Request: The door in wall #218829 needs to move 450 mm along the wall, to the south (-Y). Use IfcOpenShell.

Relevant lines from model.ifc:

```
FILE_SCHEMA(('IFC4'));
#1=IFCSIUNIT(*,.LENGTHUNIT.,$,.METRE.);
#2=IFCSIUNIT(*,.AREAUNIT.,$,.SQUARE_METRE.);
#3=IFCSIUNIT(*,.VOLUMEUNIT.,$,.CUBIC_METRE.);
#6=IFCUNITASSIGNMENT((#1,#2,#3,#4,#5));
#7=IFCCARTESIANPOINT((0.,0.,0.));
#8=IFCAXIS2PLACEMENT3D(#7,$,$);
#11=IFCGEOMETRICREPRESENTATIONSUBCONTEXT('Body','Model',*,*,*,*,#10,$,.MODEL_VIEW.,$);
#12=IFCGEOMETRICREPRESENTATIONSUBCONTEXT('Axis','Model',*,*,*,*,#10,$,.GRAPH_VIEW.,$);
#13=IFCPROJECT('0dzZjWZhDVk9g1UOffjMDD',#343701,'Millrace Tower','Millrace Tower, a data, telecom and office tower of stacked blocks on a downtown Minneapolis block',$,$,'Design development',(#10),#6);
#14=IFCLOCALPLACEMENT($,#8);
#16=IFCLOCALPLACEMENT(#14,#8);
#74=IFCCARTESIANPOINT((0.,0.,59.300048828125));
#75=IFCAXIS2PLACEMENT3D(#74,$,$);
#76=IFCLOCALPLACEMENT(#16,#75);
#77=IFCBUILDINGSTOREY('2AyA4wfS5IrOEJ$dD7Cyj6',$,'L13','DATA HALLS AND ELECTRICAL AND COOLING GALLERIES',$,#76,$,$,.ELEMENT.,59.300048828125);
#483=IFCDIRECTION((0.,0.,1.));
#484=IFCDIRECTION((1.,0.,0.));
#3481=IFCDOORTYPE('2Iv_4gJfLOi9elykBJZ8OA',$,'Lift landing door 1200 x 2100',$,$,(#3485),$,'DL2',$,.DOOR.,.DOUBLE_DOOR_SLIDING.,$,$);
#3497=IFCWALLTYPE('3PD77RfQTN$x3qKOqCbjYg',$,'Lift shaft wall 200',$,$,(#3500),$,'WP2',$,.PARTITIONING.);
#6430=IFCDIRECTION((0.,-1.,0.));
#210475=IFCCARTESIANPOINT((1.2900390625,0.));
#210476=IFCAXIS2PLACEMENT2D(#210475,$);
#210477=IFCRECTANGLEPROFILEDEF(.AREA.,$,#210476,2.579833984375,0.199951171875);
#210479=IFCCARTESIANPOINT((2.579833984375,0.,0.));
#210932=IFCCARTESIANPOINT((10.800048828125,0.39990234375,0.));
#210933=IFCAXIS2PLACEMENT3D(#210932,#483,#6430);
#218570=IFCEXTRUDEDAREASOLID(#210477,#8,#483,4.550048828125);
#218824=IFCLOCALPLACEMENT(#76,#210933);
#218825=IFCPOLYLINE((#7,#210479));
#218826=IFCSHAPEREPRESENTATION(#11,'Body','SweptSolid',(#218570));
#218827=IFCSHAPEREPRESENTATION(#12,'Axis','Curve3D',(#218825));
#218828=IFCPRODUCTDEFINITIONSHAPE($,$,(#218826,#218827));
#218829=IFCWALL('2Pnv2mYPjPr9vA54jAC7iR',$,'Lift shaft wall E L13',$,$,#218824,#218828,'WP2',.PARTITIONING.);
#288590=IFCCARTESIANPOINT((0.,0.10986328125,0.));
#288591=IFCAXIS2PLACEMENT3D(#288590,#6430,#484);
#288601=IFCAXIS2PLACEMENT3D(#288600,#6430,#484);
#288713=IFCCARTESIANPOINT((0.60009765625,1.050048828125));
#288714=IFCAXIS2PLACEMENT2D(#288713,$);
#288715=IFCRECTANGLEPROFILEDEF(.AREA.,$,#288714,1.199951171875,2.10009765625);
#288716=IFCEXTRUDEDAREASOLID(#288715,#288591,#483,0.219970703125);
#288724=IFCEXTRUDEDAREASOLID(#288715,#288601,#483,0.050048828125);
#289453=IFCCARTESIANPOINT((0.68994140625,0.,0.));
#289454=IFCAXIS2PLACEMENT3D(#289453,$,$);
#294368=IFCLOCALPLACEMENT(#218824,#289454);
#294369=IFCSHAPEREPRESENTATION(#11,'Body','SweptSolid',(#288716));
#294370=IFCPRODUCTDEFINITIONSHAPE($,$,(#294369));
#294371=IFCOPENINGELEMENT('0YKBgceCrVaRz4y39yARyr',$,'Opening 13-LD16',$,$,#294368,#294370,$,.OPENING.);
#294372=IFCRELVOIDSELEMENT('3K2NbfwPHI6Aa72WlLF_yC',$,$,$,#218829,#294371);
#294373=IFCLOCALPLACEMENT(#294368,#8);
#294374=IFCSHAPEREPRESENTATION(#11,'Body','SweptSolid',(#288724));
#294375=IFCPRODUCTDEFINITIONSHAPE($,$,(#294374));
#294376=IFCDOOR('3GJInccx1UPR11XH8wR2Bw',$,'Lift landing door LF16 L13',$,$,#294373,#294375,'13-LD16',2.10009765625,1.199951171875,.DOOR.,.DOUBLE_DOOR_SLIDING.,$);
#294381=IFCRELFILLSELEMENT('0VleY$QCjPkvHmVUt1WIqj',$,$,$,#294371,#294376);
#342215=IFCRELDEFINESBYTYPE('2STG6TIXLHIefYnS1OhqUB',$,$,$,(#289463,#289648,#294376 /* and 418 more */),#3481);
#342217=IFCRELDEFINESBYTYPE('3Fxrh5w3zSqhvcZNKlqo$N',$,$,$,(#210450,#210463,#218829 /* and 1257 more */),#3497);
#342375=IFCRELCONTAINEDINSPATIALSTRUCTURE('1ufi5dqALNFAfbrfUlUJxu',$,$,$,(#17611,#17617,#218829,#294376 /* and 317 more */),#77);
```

```python
import ifcopenshell
import ifcopenshell.api.geometry
import ifcopenshell.util.placement

model = ifcopenshell.open("model.ifc")

door = model.by_guid("3GJInccx1UPR11XH8wR2Bw")
opening = door.FillsVoids[0].RelatingOpeningElement
wall = opening.VoidsElements[0].RelatingBuildingElement

wall_matrix = ifcopenshell.util.placement.get_local_placement(wall.ObjectPlacement)
shift = wall_matrix[:3, 0] * 0.45
before = ifcopenshell.util.placement.get_local_placement(door.ObjectPlacement)[:3, 3].copy()

# The door is placed relative to its opening, so it follows when the opening moves.
matrix = ifcopenshell.util.placement.get_local_placement(opening.ObjectPlacement)
matrix[:3, 3] += shift
ifcopenshell.api.geometry.edit_object_placement(
    model, product=opening, matrix=matrix, is_si=False, should_transform_children=True
)

after = ifcopenshell.util.placement.get_local_placement(door.ObjectPlacement)[:3, 3]
print("door moved by", (after - before).round(3) + 0.0)

model.write("model-out.ifc")
```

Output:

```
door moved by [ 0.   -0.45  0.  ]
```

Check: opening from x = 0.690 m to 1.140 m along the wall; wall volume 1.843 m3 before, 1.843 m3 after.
